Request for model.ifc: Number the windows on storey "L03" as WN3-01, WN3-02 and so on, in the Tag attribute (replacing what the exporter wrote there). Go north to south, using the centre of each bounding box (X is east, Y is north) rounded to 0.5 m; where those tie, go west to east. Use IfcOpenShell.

First a look at what the model holds.

```python
import ifcopenshell
import ifcopenshell.util.element
import ifcopenshell.util.placement

model = ifcopenshell.open("model.ifc")
print(model.schema)
storey = next(s for s in model.by_type("IfcBuildingStorey") if s.Name == "L03")
windows = [e for e in ifcopenshell.util.element.get_decomposition(storey) if e.is_a("IfcWindow")]
for e in sorted(windows, key=lambda e: e.id()):
    origin = ifcopenshell.util.placement.get_local_placement(e.ObjectPlacement)[:3, 3]
    print(e.id(), e.Tag, e.Name, origin.round(2) + 0.0, sep=" | ")
```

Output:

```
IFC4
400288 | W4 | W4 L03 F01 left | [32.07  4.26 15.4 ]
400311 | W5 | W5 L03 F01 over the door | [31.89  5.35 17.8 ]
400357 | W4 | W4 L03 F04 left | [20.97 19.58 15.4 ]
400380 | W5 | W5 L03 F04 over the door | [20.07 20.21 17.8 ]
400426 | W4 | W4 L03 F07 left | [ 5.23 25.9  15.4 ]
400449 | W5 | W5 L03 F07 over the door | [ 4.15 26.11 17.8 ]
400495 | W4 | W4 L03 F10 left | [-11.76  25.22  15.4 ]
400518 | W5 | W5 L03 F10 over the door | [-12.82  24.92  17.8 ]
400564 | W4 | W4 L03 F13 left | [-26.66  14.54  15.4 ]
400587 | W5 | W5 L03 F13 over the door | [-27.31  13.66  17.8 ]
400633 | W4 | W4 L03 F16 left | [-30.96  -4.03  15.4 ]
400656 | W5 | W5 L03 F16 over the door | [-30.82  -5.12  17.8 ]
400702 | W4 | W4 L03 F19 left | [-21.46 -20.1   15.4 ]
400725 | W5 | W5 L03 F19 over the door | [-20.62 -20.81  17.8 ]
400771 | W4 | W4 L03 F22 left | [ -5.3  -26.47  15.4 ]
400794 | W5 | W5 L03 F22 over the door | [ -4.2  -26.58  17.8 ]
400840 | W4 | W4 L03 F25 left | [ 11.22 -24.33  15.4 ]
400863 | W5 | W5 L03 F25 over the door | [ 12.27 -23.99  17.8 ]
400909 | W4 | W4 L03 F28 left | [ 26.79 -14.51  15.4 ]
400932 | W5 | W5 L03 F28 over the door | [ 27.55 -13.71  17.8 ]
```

```python
import ifcopenshell
import ifcopenshell.geom
import ifcopenshell.util.element
import ifcopenshell.util.shape

model = ifcopenshell.open("model.ifc")
settings = ifcopenshell.geom.settings()
settings.set("use-world-coords", True)


def centre(element):
    shape = ifcopenshell.geom.create_shape(settings, element)
    return ifcopenshell.util.shape.get_bbox_centroid(shape.geometry)


storey = next(s for s in model.by_type("IfcBuildingStorey") if s.Name == "L03")
windows = [e for e in ifcopenshell.util.element.get_decomposition(storey) if e.is_a("IfcWindow")]

# Insertion points can sit at a corner or the storey origin, so sort by the geometry (in metres).
centres = {e: centre(e) for e in windows}
windows.sort(key=lambda e: (-round(centres[e][1] / 0.5), centres[e][0]))

for i, e in enumerate(windows, start=1):
    number = f"WN3-{i:02d}"
    e.Tag = number
    print(e.id(), number)

model.write("model_rev.ifc")
```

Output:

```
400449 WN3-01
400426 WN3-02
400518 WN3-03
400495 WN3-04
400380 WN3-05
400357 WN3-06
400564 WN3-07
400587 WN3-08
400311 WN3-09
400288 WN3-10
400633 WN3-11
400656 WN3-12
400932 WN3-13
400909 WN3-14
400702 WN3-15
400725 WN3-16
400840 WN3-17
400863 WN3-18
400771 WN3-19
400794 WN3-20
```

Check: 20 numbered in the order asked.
